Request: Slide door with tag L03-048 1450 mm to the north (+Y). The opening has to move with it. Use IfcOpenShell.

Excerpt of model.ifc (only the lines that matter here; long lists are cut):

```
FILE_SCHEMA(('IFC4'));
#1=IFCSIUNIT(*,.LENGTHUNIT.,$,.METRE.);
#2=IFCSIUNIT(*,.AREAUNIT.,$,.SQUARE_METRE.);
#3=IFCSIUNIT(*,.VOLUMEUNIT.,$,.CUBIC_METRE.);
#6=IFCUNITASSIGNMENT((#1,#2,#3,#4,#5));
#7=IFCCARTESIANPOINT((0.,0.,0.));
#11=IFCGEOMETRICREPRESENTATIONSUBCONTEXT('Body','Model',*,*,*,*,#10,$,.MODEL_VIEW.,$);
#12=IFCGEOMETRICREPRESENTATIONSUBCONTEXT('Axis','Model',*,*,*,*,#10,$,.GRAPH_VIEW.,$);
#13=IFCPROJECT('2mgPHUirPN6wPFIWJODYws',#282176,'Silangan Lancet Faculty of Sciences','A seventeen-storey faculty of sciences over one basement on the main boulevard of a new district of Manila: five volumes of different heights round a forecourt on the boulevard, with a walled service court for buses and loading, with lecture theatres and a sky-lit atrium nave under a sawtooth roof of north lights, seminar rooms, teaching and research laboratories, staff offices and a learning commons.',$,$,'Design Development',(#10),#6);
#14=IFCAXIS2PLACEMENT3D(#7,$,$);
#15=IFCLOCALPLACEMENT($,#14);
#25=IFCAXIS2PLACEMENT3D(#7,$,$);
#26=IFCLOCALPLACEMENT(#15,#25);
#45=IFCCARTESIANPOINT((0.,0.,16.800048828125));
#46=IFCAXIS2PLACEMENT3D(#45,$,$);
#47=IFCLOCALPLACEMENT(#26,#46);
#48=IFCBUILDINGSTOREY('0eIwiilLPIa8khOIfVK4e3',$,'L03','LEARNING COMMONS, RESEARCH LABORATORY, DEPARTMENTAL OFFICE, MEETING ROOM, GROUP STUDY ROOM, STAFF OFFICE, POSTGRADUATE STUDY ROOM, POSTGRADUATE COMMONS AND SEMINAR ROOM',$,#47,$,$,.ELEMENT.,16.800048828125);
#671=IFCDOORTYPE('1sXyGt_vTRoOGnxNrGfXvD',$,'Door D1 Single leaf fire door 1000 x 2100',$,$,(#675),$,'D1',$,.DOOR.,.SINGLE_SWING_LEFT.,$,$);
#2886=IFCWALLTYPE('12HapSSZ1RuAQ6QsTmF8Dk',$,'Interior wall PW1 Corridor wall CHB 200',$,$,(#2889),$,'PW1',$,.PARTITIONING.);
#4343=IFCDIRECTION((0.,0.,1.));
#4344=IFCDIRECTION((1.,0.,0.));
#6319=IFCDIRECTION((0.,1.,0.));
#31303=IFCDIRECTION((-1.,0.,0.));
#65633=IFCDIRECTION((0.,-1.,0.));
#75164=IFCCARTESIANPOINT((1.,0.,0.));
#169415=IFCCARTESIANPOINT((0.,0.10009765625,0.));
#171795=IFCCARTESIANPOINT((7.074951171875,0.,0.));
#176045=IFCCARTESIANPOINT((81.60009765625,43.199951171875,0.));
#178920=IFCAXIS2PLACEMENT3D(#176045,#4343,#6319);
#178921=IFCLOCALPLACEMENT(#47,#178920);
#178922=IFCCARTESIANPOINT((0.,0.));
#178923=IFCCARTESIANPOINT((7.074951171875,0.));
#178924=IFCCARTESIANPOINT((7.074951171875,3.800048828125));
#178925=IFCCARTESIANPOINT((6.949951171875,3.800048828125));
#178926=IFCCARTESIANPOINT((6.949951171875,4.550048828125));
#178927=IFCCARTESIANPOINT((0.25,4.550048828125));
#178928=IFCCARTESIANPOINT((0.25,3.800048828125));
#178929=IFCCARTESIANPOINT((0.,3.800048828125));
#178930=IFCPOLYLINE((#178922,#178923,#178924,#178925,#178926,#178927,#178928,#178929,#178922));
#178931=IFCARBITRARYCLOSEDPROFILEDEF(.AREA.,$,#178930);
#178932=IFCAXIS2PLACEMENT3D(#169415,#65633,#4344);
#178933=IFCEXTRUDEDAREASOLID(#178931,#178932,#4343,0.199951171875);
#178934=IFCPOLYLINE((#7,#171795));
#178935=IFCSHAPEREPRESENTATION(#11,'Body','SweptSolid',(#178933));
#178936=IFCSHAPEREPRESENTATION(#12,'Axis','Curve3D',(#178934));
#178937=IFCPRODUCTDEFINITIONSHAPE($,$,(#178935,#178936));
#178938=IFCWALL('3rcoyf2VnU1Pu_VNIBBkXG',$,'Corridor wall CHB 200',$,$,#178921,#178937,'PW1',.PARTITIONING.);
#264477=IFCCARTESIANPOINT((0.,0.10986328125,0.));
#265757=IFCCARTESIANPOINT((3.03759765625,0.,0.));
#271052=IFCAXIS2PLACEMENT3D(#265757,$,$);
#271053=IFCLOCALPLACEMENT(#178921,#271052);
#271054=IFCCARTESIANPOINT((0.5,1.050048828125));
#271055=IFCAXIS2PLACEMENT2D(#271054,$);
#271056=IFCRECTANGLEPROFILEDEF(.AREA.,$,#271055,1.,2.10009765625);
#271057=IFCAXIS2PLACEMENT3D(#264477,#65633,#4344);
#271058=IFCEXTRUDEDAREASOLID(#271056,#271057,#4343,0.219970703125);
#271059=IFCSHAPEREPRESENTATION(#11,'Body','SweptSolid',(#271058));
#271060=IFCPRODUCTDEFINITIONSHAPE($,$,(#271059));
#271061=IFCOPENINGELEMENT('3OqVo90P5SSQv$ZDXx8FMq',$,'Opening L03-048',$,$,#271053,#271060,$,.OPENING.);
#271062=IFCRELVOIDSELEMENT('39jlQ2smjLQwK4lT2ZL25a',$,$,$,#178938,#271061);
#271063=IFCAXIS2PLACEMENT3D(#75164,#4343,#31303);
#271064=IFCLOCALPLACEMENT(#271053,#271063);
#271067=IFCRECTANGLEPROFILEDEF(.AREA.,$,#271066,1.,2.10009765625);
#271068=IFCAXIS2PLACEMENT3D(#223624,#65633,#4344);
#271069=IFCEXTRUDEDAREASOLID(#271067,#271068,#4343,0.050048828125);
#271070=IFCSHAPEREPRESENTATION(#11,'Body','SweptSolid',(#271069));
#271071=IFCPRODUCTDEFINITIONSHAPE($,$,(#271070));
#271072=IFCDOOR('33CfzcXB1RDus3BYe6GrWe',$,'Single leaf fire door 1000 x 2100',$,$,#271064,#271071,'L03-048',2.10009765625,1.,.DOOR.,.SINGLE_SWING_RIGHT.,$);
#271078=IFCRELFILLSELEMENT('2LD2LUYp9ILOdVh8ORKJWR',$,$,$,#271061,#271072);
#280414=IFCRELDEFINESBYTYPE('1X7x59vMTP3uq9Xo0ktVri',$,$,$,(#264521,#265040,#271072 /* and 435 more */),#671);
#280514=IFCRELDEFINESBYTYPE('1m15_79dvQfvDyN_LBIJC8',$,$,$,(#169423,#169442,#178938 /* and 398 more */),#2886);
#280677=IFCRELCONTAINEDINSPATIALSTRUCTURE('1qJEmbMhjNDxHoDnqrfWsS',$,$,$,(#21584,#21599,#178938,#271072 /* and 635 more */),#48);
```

```python
import ifcopenshell
import ifcopenshell.api.geometry
import ifcopenshell.util.placement
import ifcopenshell.util.unit

model = ifcopenshell.open("model.ifc")
unit_scale = ifcopenshell.util.unit.calculate_unit_scale(model)

door = model.by_guid("33CfzcXB1RDus3BYe6GrWe")
opening = door.FillsVoids[0].RelatingOpeningElement
wall = opening.VoidsElements[0].RelatingBuildingElement

wall_matrix = ifcopenshell.util.placement.get_local_placement(wall.ObjectPlacement)
shift = wall_matrix[:3, 0] * 1.45 / unit_scale
before = ifcopenshell.util.placement.get_local_placement(door.ObjectPlacement)[:3, 3].copy()

# The door is placed relative to its opening, so it follows when the opening moves.
matrix = ifcopenshell.util.placement.get_local_placement(opening.ObjectPlacement)
matrix[:3, 3] += shift
ifcopenshell.api.geometry.edit_object_placement(
    model, product=opening, matrix=matrix, is_si=False, should_transform_children=True
)

after = ifcopenshell.util.placement.get_local_placement(door.ObjectPlacement)[:3, 3]
print("door moved by", (after - before).round(3) + 0.0)

model.write("model_rev.ifc")
```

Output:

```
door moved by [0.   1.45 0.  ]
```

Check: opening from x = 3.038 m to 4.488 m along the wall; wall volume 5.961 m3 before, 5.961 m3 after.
